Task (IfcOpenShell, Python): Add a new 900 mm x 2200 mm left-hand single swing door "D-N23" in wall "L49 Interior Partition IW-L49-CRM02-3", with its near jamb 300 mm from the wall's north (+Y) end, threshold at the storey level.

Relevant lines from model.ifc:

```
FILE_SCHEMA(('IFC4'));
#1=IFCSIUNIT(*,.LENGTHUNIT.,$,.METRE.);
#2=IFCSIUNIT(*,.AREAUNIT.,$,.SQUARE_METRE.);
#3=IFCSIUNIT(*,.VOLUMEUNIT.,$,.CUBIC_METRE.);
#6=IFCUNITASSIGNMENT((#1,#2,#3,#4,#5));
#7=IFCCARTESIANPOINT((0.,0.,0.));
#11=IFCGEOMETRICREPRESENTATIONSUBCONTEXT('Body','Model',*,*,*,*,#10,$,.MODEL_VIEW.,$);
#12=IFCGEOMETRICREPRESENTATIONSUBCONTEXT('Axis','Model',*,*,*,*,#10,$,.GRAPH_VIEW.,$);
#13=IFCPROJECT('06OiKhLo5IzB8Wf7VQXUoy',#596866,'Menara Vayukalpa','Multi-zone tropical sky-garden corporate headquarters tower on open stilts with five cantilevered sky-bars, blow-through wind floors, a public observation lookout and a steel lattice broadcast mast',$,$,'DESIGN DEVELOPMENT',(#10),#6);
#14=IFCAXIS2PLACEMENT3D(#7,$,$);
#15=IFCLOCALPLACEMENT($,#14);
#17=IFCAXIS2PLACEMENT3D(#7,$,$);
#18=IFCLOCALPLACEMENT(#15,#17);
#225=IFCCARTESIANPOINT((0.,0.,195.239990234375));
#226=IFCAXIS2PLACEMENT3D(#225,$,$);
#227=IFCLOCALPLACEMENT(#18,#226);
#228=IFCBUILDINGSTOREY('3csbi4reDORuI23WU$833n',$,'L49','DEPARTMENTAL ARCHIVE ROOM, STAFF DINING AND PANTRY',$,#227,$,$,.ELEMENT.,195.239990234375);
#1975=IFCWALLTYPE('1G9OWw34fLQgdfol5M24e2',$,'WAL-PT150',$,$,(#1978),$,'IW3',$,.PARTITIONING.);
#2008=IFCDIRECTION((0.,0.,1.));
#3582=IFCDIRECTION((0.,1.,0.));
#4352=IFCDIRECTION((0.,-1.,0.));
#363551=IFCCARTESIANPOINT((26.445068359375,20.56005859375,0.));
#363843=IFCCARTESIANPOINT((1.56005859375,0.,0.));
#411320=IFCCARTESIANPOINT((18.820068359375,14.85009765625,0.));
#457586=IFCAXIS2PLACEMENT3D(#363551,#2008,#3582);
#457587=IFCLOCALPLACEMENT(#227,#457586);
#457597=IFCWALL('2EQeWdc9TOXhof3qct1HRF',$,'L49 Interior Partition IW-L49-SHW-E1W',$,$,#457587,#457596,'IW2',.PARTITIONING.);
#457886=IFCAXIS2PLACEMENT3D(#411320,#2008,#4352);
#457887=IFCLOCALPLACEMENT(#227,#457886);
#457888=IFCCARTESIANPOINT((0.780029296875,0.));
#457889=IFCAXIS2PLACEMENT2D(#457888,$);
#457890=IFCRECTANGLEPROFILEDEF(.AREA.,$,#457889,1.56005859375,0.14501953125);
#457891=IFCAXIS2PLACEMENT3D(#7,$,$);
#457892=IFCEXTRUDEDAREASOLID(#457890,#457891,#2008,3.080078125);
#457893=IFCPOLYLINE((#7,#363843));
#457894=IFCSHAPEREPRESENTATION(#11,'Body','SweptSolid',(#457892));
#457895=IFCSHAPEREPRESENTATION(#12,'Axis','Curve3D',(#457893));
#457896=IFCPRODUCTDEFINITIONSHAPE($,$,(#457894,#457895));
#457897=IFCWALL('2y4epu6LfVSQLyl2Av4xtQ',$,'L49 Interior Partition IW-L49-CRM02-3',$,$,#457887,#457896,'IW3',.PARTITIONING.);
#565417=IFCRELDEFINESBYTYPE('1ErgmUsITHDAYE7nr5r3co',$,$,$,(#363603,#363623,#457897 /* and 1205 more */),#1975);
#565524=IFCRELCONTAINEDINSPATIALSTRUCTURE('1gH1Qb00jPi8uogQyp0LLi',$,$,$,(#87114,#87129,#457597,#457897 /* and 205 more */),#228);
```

```python
import numpy as np
import ifcopenshell
import ifcopenshell.api.feature
import ifcopenshell.api.geometry
import ifcopenshell.api.root
import ifcopenshell.api.spatial
import ifcopenshell.geom
import ifcopenshell.util.element
import ifcopenshell.util.placement
import ifcopenshell.util.representation
import ifcopenshell.util.shape
import ifcopenshell.util.unit

model = ifcopenshell.open("model.ifc")
unit_scale = ifcopenshell.util.unit.calculate_unit_scale(model)
settings = ifcopenshell.geom.settings()


def volume(element):
    """Net volume in cubic metres, openings subtracted."""
    shape = ifcopenshell.geom.create_shape(settings, element)
    return ifcopenshell.util.shape.get_volume(shape.geometry)


wall = model.by_guid("2y4epu6LfVSQLyl2Av4xtQ")
storey = ifcopenshell.util.element.get_container(wall, ifc_class="IfcBuildingStorey")
context = ifcopenshell.util.representation.get_context(model, "Model", "Body", "MODEL_VIEW")
before = volume(wall)

width, height, from_end, sill = 0.9, 2.2, 0.3, 0.0  # metres

# The wall runs along its own X axis, and the end named is its -X end.
wall_shape = ifcopenshell.geom.create_shape(settings, wall)
x, y, z = ifcopenshell.util.shape.get_vertices(wall_shape.geometry).T
start = x.min() + from_end
face, thickness = float(y.min()), float(y.max() - y.min())
wall_matrix = ifcopenshell.util.placement.get_local_placement(wall.ObjectPlacement)
level = ifcopenshell.util.placement.get_local_placement(storey.ObjectPlacement)[2, 3]


def in_wall(x, y):
    """Placement at x, y metres in the wall's axes, at sill height."""
    matrix = wall_matrix.copy()
    matrix[:, 3] = wall_matrix @ np.array([x / unit_scale, y / unit_scale, 0.0, 1.0])
    matrix[2, 3] = level + sill / unit_scale
    return matrix


# Opening: a box that overshoots both wall faces by 50 mm.
opening = ifcopenshell.api.root.create_entity(model, ifc_class="IfcOpeningElement", predefined_type="OPENING")
box = ifcopenshell.api.geometry.add_wall_representation(
    model, context=context, length=width, height=height, thickness=thickness + 0.1
)
ifcopenshell.api.geometry.assign_representation(model, product=opening, representation=box)
ifcopenshell.api.geometry.edit_object_placement(model, product=opening, matrix=in_wall(start, face - 0.05), is_si=False)
ifcopenshell.api.feature.add_feature(model, feature=opening, element=wall)

door = ifcopenshell.api.root.create_entity(model, ifc_class="IfcDoor", name="D-N23", predefined_type="DOOR")
door.OverallWidth, door.OverallHeight = width / unit_scale, height / unit_scale
door.OperationType = "SINGLE_SWING_LEFT"
body = ifcopenshell.api.geometry.add_door_representation(
    model,
    context=context,
    overall_width=door.OverallWidth,
    overall_height=door.OverallHeight,
    operation_type="SINGLE_SWING_LEFT",
    lining_properties={"LiningDepth": thickness / unit_scale, "ThresholdDepth": thickness / unit_scale},
)
ifcopenshell.api.geometry.assign_representation(model, product=door, representation=body)
ifcopenshell.api.spatial.assign_container(model, products=[door], relating_structure=storey)
ifcopenshell.api.feature.add_filling(model, opening=opening, element=door)

# The lining spans the wall, so the door starts at the wall face.
ifcopenshell.api.geometry.edit_object_placement(model, product=door, matrix=in_wall(start, face), is_si=False)

after = volume(wall)

print(f"wall volume {before:.3f} -> {after:.3f} m3")

model.write("model_edited.ifc")
```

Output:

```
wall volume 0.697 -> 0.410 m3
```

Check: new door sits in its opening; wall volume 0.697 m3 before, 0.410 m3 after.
